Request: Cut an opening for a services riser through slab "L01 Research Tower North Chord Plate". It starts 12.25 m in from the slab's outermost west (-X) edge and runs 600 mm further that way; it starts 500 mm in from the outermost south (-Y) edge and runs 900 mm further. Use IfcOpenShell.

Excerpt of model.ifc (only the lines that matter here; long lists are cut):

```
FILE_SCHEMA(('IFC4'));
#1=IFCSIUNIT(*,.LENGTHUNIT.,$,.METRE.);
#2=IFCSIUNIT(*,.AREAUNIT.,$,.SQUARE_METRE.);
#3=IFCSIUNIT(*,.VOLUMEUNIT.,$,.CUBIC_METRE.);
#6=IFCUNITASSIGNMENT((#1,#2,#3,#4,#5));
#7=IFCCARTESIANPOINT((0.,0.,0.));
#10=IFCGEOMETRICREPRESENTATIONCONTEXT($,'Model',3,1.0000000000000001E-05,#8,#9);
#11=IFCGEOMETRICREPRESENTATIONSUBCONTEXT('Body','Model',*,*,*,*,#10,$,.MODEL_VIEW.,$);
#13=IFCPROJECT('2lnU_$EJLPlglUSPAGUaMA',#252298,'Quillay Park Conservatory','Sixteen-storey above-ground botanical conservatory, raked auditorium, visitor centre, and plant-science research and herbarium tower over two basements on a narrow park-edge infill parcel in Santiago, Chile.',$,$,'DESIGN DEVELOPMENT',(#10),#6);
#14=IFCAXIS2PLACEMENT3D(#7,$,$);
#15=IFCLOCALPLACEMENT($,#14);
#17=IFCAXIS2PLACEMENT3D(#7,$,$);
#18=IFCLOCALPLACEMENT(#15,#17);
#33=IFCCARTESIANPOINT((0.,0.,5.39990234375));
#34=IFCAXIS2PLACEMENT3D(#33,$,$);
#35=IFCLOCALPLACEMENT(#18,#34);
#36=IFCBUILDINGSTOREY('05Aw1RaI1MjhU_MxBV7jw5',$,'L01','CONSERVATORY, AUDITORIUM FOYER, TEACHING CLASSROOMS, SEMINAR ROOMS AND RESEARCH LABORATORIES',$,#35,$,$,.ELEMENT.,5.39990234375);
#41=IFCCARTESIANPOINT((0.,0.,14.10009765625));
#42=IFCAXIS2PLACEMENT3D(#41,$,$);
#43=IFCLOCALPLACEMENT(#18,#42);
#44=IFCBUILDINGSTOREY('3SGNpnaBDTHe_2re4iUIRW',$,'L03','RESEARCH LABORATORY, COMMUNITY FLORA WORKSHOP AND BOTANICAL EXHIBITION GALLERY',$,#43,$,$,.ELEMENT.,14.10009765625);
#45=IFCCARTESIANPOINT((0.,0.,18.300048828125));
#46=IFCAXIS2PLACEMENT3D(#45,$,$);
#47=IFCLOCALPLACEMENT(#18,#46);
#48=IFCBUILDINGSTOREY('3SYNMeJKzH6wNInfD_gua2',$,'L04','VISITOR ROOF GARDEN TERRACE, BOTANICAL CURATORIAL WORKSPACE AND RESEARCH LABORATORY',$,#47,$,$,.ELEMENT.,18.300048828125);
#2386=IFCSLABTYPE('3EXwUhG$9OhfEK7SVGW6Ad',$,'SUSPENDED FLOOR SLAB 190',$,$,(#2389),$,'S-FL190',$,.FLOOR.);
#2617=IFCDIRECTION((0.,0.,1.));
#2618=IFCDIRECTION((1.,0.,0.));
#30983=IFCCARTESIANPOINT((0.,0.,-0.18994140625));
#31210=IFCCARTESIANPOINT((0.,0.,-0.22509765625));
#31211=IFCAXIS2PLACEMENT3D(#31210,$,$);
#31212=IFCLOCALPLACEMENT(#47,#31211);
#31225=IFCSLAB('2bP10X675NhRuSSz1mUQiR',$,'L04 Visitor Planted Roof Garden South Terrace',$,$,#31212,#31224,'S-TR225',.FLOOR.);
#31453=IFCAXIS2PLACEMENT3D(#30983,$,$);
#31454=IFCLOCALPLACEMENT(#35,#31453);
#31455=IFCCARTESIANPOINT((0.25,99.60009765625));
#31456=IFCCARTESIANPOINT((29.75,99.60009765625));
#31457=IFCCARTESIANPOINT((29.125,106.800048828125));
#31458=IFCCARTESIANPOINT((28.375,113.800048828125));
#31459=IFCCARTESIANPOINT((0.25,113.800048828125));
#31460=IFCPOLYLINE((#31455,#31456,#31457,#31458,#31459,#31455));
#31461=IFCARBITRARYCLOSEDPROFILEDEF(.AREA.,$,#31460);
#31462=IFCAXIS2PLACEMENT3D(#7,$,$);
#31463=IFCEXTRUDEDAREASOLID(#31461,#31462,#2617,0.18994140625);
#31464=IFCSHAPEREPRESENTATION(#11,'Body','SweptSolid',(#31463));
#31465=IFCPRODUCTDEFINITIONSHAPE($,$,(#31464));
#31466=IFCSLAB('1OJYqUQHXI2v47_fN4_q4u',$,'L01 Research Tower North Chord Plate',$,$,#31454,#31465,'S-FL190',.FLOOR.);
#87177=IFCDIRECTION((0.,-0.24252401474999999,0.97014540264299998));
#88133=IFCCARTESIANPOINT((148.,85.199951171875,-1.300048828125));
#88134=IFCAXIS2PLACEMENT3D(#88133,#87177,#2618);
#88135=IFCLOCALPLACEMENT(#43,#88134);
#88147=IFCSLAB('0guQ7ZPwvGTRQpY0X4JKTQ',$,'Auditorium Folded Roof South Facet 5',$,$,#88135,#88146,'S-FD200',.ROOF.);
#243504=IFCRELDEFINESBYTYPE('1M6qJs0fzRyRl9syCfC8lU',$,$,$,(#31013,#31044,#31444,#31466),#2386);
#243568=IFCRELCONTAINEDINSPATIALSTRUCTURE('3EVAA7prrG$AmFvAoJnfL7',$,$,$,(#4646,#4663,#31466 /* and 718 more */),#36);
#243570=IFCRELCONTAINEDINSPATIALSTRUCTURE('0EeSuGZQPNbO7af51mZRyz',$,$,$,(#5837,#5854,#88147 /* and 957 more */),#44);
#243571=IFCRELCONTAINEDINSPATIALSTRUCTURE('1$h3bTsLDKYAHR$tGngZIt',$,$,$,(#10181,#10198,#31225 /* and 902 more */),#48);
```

```python
import numpy as np
import ifcopenshell
import ifcopenshell.api.feature
import ifcopenshell.api.geometry
import ifcopenshell.api.root
import ifcopenshell.geom
import ifcopenshell.util.placement
import ifcopenshell.util.representation
import ifcopenshell.util.shape
import ifcopenshell.util.unit

model = ifcopenshell.open("model.ifc")
unit_scale = ifcopenshell.util.unit.calculate_unit_scale(model)
settings = ifcopenshell.geom.settings()


def volume(element):
    """Net volume in cubic metres, openings subtracted."""
    shape = ifcopenshell.geom.create_shape(settings, element)
    return ifcopenshell.util.shape.get_volume(shape.geometry)


slab = model.by_guid("1OJYqUQHXI2v47_fN4_q4u")
before = volume(slab)

# Extent in the slab's own axes, in metres. The edges named are its -X and -Y sides.
slab_shape = ifcopenshell.geom.create_shape(settings, slab)
vertices = ifcopenshell.util.shape.get_vertices(slab_shape.geometry)
x_min, y_min, bottom = vertices.min(axis=0)
top = vertices[:, 2].max()

opening = ifcopenshell.api.root.create_entity(model, ifc_class="IfcOpeningElement", name="Services riser opening", predefined_type="OPENING")
context = ifcopenshell.util.representation.get_context(model, "Model", "Body", "MODEL_VIEW")
width, depth = 0.6, 0.9
outline = [(0.0, 0.0), (width, 0.0), (width, depth), (0.0, depth), (0.0, 0.0)]
# Overshoot both faces by 50 mm so the cut is clean.
shape = ifcopenshell.api.geometry.add_slab_representation(
    model, context=context, depth=top - bottom + 0.1, polyline=outline
)
ifcopenshell.api.geometry.assign_representation(model, product=opening, representation=shape)

matrix = ifcopenshell.util.placement.get_local_placement(slab.ObjectPlacement)
matrix[:, 3] = matrix @ np.append(np.array([x_min + 12.25, y_min + 0.5, bottom - 0.05]) / unit_scale, 1.0)
ifcopenshell.api.geometry.edit_object_placement(model, product=opening, matrix=matrix, is_si=False)
ifcopenshell.api.feature.add_feature(model, feature=opening, element=slab)

after = volume(slab)

print(f"slab volume {before:.3f} -> {after:.3f} m3")

model.write("model_rev.ifc")
```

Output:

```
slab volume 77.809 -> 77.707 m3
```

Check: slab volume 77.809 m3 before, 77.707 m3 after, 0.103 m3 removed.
